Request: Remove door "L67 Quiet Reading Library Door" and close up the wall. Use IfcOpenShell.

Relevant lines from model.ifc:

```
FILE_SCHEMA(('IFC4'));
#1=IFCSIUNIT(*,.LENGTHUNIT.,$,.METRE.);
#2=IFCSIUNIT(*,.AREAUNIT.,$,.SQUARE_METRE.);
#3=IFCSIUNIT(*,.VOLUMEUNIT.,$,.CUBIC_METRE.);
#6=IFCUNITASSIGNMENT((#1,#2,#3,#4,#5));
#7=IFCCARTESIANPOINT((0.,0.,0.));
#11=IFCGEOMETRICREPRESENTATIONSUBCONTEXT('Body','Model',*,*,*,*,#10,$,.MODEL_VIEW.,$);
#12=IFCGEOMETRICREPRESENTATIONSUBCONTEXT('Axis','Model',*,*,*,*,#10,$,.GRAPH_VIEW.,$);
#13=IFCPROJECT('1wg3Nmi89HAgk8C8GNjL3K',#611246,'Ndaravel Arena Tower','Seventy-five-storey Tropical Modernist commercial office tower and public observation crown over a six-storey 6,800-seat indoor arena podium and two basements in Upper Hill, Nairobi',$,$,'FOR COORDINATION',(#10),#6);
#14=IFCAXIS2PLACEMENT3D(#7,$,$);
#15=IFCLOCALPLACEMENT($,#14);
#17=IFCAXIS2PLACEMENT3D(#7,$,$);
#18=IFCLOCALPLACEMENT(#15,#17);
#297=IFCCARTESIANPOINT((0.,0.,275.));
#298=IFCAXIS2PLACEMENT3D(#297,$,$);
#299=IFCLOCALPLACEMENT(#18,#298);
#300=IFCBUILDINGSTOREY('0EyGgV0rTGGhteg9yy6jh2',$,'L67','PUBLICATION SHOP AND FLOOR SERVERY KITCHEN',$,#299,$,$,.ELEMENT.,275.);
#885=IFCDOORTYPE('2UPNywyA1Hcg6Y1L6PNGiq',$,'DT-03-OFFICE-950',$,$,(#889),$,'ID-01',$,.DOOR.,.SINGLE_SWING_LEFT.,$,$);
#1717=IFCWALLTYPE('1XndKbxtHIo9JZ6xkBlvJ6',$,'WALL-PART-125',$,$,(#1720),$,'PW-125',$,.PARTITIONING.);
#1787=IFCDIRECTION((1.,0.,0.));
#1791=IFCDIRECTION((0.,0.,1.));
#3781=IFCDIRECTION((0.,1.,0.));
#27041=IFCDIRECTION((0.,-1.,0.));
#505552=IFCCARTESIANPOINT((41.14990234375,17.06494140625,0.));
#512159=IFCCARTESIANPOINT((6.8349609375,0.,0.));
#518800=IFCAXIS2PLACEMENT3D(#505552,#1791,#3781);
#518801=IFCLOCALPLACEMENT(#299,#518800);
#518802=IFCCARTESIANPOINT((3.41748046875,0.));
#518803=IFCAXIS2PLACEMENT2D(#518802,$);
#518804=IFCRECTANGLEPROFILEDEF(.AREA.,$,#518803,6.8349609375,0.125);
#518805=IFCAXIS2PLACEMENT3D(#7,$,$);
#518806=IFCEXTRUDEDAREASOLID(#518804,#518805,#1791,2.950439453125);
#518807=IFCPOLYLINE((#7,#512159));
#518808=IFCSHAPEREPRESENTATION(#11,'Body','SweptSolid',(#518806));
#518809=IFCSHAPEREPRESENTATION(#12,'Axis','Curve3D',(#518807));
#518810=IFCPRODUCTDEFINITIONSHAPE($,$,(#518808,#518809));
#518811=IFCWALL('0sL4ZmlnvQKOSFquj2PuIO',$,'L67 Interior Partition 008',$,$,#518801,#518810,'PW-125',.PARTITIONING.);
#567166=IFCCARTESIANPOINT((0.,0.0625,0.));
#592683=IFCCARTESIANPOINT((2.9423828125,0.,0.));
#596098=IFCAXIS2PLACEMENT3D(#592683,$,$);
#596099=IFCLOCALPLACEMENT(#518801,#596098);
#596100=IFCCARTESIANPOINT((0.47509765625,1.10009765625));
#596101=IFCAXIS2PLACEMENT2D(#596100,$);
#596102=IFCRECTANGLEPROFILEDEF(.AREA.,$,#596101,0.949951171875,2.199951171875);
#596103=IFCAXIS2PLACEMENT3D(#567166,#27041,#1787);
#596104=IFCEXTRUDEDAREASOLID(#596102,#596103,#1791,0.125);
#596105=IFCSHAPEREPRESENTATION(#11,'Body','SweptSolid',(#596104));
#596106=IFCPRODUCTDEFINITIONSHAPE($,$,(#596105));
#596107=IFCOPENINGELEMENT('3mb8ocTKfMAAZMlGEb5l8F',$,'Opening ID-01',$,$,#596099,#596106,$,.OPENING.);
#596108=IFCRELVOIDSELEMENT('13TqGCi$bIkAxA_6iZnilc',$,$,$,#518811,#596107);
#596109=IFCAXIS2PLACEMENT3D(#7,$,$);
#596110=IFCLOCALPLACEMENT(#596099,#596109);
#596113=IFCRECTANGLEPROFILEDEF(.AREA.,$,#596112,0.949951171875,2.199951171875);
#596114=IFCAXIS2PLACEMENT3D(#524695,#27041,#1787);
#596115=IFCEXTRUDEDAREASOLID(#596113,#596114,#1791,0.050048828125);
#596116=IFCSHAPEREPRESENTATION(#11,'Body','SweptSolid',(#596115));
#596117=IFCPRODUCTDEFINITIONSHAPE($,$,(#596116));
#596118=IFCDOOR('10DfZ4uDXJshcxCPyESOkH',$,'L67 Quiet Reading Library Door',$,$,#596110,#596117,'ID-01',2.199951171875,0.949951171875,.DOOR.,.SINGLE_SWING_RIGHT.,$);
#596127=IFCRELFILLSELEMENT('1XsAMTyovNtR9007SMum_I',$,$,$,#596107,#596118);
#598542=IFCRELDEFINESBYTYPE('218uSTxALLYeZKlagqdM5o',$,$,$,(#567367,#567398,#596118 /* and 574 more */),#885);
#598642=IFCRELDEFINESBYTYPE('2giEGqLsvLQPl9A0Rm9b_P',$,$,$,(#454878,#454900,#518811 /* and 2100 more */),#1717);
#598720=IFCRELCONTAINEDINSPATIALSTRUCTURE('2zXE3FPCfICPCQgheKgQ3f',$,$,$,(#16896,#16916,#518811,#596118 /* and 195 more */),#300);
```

```python
import ifcopenshell
import ifcopenshell.api.feature
import ifcopenshell.api.root
import ifcopenshell.geom
import ifcopenshell.util.shape

model = ifcopenshell.open("model.ifc")
settings = ifcopenshell.geom.settings()


def volume(element):
    """Net volume in cubic metres, openings subtracted."""
    shape = ifcopenshell.geom.create_shape(settings, element)
    return ifcopenshell.util.shape.get_volume(shape.geometry)


door = model.by_id(596118)
opening = door.FillsVoids[0].RelatingOpeningElement
wall = opening.VoidsElements[0].RelatingBuildingElement
before = volume(wall)

ifcopenshell.api.root.remove_product(model, product=door)
ifcopenshell.api.feature.remove_feature(model, feature=opening)

after = volume(wall)

print(f"wall volume {before:.3f} -> {after:.3f} m3")

model.write("model-out.ifc")
```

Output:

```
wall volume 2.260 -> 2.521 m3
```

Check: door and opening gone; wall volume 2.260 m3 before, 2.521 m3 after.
